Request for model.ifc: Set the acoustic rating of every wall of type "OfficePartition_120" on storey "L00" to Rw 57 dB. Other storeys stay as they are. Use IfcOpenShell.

First a look at what the model holds.

```python
import ifcopenshell
import ifcopenshell.util.element

model = ifcopenshell.open("model.ifc")
print(model.schema)
storey = next(s for s in model.by_type("IfcBuildingStorey") if s.Name == "L00")
walls = [e for e in ifcopenshell.util.element.get_decomposition(storey) if e.is_a("IfcWall")]
seen = {}
for e in walls:
    element_type = ifcopenshell.util.element.get_type(e)
    key = (element_type.Name if element_type != e and element_type else None, ifcopenshell.util.element.get_pset(e, "Pset_WallCommon", "AcousticRating"))
    seen[key] = seen.get(key, 0) + 1
for (name, value), count in sorted(seen.items(), key=str):
    print(count, "x", name, "|", value)
```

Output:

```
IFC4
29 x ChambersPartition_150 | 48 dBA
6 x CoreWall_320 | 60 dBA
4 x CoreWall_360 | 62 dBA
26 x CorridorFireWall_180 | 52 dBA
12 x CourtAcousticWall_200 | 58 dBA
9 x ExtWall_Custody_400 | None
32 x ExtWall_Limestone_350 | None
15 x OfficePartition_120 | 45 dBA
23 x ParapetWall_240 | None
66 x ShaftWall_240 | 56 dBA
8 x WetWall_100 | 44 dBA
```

```python
import ifcopenshell
import ifcopenshell.api.pset
import ifcopenshell.util.element

model = ifcopenshell.open("model.ifc")

storey = next(s for s in model.by_type("IfcBuildingStorey") if s.Name == "L00")
walls = [e for e in ifcopenshell.util.element.get_decomposition(storey) if e.is_a("IfcWall")]

count = 0
for e in walls:
    element_type = ifcopenshell.util.element.get_type(e)
    if element_type in (None, e) or element_type.Name != "OfficePartition_120":
        continue
    # add_pset returns the element's existing set when there is one.
    pset = ifcopenshell.api.pset.add_pset(model, product=e, name="Pset_WallCommon")
    ifcopenshell.api.pset.edit_pset(model, pset=pset, properties={"AcousticRating": "Rw 57 dB"})
    count += 1

print(count, "walls updated")

model.write("model_edited.ifc")
```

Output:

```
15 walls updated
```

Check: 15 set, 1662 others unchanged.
